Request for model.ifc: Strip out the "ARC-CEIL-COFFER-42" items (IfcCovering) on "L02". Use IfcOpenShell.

First a look at what the model holds.

```python
import ifcopenshell
import ifcopenshell.util.element

model = ifcopenshell.open("model.ifc")
print(model.schema)
storey = next(s for s in model.by_type("IfcBuildingStorey") if s.Name == "L02")
coverings = [e for e in ifcopenshell.util.element.get_decomposition(storey) if e.is_a("IfcCovering")]
seen = {}
for e in coverings:
    element_type = ifcopenshell.util.element.get_type(e)
    name = element_type.Name if element_type not in (None, e) else None
    seen[name] = seen.get(name, 0) + 1
for name, count in sorted(seen.items(), key=str):
    print(count, "x", name)
```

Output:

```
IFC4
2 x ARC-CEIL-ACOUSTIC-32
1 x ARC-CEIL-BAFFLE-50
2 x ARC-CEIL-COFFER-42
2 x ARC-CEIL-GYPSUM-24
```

```python
import ifcopenshell
import ifcopenshell.api.root
import ifcopenshell.util.element

model = ifcopenshell.open("model.ifc")

storey = next(s for s in model.by_type("IfcBuildingStorey") if s.Name == "L02")
coverings = [e for e in ifcopenshell.util.element.get_decomposition(storey) if e.is_a("IfcCovering")]
targets = [e for e in coverings if (t := ifcopenshell.util.element.get_type(e)) not in (None, e) and t.Name == "ARC-CEIL-COFFER-42"]

for e in targets:
    ifcopenshell.api.root.remove_product(model, product=e)
print(len(targets), "removed")

model.write("model_updated.ifc")
```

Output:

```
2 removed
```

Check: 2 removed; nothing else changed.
